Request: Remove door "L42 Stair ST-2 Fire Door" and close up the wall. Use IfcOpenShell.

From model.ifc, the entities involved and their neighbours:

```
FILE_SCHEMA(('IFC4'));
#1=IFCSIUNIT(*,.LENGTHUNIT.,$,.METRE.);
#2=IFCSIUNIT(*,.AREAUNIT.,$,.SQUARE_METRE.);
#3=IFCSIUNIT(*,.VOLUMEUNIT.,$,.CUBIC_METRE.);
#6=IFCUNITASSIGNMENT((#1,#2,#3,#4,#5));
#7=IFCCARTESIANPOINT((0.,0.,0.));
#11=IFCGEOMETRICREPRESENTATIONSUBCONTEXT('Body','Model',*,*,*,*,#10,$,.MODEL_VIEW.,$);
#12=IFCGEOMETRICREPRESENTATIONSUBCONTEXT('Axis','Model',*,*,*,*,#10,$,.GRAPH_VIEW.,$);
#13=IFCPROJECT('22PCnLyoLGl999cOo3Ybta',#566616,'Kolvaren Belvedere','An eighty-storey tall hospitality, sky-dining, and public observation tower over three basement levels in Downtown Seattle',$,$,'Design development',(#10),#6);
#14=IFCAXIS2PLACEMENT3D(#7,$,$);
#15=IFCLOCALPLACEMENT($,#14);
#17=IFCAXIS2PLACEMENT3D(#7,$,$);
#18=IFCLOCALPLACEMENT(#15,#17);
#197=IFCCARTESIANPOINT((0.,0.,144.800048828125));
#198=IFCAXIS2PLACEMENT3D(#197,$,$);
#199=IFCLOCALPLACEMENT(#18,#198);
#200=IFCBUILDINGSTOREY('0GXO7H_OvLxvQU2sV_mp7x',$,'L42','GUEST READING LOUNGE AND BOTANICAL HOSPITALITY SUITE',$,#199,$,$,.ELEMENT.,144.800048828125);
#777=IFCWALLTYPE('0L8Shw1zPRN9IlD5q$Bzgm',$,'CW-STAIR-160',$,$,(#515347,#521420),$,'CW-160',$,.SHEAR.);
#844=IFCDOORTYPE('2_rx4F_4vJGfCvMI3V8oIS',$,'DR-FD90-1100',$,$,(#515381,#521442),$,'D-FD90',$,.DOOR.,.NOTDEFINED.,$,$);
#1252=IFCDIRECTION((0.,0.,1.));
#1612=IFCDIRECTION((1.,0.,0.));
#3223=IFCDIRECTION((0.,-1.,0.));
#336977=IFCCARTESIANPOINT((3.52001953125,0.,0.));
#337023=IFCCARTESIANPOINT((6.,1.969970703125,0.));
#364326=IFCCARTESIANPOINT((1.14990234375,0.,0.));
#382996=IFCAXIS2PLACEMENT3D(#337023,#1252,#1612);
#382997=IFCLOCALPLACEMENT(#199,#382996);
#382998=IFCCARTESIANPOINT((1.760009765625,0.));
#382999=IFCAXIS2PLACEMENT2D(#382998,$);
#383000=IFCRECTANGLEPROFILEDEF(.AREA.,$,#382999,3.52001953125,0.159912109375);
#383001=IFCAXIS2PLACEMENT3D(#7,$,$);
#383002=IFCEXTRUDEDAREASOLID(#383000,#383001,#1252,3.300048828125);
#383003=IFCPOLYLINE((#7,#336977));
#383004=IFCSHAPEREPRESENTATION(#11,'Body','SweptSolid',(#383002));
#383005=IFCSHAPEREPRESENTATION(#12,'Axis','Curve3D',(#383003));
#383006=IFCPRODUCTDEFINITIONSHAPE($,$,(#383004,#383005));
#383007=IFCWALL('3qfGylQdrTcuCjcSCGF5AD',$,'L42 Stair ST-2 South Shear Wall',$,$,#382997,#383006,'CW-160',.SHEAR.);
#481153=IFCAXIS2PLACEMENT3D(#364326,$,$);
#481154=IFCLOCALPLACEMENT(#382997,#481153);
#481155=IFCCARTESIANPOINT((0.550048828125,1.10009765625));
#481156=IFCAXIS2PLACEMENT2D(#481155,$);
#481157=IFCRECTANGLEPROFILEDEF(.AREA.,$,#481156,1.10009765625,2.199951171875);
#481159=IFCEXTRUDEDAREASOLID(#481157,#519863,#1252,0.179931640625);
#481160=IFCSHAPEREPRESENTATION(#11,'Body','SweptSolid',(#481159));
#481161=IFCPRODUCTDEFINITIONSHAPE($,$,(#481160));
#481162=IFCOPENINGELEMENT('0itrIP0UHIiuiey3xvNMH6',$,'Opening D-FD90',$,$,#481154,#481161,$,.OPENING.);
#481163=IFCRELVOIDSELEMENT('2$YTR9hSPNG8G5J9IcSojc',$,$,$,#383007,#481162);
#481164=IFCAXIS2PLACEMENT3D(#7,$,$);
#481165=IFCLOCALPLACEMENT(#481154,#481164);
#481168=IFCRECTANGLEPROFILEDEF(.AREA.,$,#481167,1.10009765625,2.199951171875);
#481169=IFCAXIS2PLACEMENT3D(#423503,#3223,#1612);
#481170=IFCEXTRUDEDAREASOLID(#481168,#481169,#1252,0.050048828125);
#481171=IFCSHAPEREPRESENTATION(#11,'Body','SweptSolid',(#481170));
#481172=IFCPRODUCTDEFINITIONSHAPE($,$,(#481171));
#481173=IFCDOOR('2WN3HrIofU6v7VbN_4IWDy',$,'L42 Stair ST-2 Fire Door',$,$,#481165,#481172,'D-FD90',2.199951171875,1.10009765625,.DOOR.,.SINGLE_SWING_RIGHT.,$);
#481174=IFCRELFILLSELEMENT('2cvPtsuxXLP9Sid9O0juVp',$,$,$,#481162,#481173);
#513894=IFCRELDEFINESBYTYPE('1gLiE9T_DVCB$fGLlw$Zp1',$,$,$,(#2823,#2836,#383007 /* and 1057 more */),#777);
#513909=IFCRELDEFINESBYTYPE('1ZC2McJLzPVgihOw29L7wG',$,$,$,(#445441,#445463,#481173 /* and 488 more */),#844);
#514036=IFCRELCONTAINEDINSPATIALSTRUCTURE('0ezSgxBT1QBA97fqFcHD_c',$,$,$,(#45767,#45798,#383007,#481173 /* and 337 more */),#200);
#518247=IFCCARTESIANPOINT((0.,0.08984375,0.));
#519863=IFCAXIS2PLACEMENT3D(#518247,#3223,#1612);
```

```python
import ifcopenshell
import ifcopenshell.api.feature
import ifcopenshell.api.root
import ifcopenshell.geom
import ifcopenshell.util.shape

model = ifcopenshell.open("model.ifc")
settings = ifcopenshell.geom.settings()


def volume(element):
    """Net volume in cubic metres, openings subtracted."""
    shape = ifcopenshell.geom.create_shape(settings, element)
    return ifcopenshell.util.shape.get_volume(shape.geometry)


door = model.by_guid("2WN3HrIofU6v7VbN_4IWDy")
opening = door.FillsVoids[0].RelatingOpeningElement
wall = opening.VoidsElements[0].RelatingBuildingElement
before = volume(wall)

ifcopenshell.api.root.remove_product(model, product=door)
ifcopenshell.api.feature.remove_feature(model, feature=opening)

after = volume(wall)

print(f"wall volume {before:.3f} -> {after:.3f} m3")

model.write("model_v2.ifc")
```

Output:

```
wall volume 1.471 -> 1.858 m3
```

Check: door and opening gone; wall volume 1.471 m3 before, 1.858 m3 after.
